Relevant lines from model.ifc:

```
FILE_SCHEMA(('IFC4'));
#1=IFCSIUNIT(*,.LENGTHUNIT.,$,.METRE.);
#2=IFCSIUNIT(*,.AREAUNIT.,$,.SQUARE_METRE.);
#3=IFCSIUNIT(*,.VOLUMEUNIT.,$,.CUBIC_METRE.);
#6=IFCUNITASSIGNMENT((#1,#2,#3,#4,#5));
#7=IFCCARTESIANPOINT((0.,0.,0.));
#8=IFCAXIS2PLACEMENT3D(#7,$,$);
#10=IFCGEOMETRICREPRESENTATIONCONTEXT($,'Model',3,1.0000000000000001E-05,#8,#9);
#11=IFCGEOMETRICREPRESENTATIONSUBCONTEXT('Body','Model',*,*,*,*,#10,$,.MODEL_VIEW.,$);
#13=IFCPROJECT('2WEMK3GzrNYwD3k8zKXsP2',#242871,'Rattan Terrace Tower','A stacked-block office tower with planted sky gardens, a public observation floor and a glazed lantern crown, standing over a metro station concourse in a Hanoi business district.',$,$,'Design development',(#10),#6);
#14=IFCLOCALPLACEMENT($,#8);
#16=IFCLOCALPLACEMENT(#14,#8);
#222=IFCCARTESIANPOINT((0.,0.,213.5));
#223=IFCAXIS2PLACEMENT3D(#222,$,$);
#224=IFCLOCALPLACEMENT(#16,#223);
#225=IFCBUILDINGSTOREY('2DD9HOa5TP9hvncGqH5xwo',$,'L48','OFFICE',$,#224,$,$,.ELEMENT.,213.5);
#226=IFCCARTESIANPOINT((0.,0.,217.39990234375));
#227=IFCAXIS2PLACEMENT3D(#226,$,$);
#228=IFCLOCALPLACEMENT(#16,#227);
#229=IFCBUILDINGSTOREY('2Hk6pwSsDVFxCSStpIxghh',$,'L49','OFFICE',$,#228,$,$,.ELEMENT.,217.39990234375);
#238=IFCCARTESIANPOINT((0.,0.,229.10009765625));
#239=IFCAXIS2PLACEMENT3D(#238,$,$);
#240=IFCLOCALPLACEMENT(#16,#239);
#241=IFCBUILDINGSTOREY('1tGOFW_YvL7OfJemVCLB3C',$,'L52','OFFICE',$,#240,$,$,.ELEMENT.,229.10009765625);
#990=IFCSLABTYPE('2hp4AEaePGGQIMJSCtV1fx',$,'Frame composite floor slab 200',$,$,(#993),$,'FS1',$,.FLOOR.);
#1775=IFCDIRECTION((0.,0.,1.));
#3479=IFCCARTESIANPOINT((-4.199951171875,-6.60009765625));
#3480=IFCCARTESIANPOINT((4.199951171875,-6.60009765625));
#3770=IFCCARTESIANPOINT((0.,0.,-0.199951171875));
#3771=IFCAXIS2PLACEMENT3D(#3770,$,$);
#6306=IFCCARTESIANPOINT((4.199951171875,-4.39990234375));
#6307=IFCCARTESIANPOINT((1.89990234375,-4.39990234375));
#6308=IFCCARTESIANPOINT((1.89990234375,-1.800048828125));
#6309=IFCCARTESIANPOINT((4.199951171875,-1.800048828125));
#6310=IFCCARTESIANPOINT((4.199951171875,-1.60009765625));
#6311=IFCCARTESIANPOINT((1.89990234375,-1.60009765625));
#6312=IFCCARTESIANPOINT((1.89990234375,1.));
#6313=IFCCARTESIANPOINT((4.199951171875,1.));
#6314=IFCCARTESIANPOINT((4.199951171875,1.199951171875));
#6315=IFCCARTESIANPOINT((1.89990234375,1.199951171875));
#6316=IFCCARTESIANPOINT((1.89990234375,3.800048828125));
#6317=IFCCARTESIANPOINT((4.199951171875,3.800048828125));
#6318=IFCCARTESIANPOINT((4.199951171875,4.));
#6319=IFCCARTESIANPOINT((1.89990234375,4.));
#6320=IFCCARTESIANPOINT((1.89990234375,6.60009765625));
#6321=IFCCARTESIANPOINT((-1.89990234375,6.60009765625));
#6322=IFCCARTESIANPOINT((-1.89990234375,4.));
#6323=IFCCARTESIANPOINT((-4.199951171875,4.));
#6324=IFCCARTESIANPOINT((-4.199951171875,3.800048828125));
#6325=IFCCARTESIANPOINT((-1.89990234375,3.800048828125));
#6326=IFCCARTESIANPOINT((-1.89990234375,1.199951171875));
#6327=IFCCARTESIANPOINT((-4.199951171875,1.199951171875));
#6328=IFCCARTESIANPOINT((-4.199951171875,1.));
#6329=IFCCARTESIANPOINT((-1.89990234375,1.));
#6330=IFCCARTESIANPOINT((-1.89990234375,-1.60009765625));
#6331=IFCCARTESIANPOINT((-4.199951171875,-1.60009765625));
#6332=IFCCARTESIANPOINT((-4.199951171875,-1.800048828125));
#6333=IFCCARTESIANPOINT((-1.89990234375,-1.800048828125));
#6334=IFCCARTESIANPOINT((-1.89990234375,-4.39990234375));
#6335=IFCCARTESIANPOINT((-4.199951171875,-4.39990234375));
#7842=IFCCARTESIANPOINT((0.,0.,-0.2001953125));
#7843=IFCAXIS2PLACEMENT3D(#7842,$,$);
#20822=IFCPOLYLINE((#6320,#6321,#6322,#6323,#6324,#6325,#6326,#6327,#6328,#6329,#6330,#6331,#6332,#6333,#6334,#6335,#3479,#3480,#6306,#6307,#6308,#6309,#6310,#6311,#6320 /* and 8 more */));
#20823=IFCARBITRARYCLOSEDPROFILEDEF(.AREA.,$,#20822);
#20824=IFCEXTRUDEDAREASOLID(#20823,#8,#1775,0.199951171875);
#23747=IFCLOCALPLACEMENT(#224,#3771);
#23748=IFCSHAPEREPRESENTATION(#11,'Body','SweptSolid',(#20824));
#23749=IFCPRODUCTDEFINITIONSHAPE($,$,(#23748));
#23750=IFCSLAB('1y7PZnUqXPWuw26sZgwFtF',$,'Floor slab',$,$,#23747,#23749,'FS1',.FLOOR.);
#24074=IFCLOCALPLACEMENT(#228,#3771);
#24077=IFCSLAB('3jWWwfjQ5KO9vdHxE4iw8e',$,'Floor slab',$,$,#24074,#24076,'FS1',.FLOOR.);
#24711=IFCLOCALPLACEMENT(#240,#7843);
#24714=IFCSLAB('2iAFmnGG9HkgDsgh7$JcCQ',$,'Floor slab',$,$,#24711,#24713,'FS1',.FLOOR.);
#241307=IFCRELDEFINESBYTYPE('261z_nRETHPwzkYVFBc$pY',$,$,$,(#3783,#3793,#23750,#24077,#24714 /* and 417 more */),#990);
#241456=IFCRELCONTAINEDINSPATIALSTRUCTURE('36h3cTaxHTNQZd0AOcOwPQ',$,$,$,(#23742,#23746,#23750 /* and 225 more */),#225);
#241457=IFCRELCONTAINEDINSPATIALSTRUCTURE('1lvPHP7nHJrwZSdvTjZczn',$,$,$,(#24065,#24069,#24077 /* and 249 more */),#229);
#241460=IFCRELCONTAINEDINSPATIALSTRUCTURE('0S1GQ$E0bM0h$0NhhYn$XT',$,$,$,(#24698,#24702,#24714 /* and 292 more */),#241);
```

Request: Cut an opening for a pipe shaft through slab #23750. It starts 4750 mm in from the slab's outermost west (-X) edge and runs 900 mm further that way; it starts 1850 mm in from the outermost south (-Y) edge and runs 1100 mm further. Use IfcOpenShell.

```python
import numpy as np
import ifcopenshell
import ifcopenshell.api.feature
import ifcopenshell.api.geometry
import ifcopenshell.api.root
import ifcopenshell.geom
import ifcopenshell.util.placement
import ifcopenshell.util.representation
import ifcopenshell.util.shape
import ifcopenshell.util.unit

model = ifcopenshell.open("model.ifc")
unit_scale = ifcopenshell.util.unit.calculate_unit_scale(model)
settings = ifcopenshell.geom.settings()


def volume(element):
    """Net volume in cubic metres, openings subtracted."""
    shape = ifcopenshell.geom.create_shape(settings, element)
    return ifcopenshell.util.shape.get_volume(shape.geometry)


slab = model.by_id(23750)
before = volume(slab)

# Extent in the slab's own axes, in metres. The edges named are its -X and -Y sides.
slab_shape = ifcopenshell.geom.create_shape(settings, slab)
vertices = ifcopenshell.util.shape.get_vertices(slab_shape.geometry)
x_min, y_min, bottom = vertices.min(axis=0)
top = vertices[:, 2].max()

opening = ifcopenshell.api.root.create_entity(model, ifc_class="IfcOpeningElement", name="Pipe shaft opening", predefined_type="OPENING")
context = ifcopenshell.util.representation.get_context(model, "Model", "Body", "MODEL_VIEW")
width, depth = 0.9, 1.1
outline = [(0.0, 0.0), (width, 0.0), (width, depth), (0.0, depth), (0.0, 0.0)]
# Overshoot both faces by 50 mm so the cut is clean.
shape = ifcopenshell.api.geometry.add_slab_representation(
    model, context=context, depth=top - bottom + 0.1, polyline=outline
)
ifcopenshell.api.geometry.assign_representation(model, product=opening, representation=shape)

matrix = ifcopenshell.util.placement.get_local_placement(slab.ObjectPlacement)
matrix[:, 3] = matrix @ np.append(np.array([x_min + 4.75, y_min + 1.85, bottom - 0.05]) / unit_scale, 1.0)
ifcopenshell.api.geometry.edit_object_placement(model, product=opening, matrix=matrix, is_si=False)
ifcopenshell.api.feature.add_feature(model, feature=opening, element=slab)

after = volume(slab)

print(f"slab volume {before:.3f} -> {after:.3f} m3")

model.write("model_rev.ifc")
```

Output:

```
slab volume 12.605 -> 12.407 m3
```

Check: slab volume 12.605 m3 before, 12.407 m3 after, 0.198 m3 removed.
